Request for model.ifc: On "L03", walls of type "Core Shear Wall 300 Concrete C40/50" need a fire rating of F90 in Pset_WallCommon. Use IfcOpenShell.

First a look at what the model holds.

```python
import ifcopenshell
import ifcopenshell.util.element

model = ifcopenshell.open("model.ifc")
print(model.schema)
storey = next(s for s in model.by_type("IfcBuildingStorey") if s.Name == "L03")
walls = [e for e in ifcopenshell.util.element.get_decomposition(storey) if e.is_a("IfcWall")]
seen = {}
for e in walls:
    element_type = ifcopenshell.util.element.get_type(e)
    key = (element_type.Name if element_type != e and element_type else None, ifcopenshell.util.element.get_pset(e, "Pset_WallCommon", "FireRating"))
    seen[key] = seen.get(key, 0) + 1
for (name, value), count in sorted(seen.items(), key=str):
    print(count, "x", name, "|", value)
```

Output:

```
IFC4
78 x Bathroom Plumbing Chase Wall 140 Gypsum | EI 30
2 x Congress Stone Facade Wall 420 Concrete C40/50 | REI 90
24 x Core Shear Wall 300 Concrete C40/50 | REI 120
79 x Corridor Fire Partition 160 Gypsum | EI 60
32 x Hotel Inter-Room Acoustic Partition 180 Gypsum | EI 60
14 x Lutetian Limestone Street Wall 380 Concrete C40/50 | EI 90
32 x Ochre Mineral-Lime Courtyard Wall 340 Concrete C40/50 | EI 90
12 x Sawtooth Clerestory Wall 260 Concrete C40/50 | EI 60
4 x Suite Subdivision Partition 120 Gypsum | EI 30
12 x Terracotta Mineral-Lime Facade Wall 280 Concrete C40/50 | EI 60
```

```python
import ifcopenshell
import ifcopenshell.api.pset
import ifcopenshell.util.element

model = ifcopenshell.open("model.ifc")

storey = next(s for s in model.by_type("IfcBuildingStorey") if s.Name == "L03")
walls = [e for e in ifcopenshell.util.element.get_decomposition(storey) if e.is_a("IfcWall")]

count = 0
for e in walls:
    element_type = ifcopenshell.util.element.get_type(e)
    if element_type in (None, e) or element_type.Name != "Core Shear Wall 300 Concrete C40/50":
        continue
    # add_pset returns the element's existing set when there is one.
    pset = ifcopenshell.api.pset.add_pset(model, product=e, name="Pset_WallCommon")
    ifcopenshell.api.pset.edit_pset(model, pset=pset, properties={"FireRating": "F90"})
    count += 1

print(count, "walls updated")

model.write("model_rev.ifc")
```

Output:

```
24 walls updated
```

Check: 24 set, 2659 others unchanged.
